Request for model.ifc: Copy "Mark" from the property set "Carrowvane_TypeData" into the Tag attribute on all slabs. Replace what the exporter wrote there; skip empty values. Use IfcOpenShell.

First a look at what the model holds.

```python
import ifcopenshell
import ifcopenshell.util.element

model = ifcopenshell.open("model.ifc")
print(model.schema)
slabs = model.by_type("IfcSlab")
print(len(slabs), "slabs")
for e in slabs[:8]:
    source = ifcopenshell.util.element.get_pset(e, "Carrowvane_TypeData", "Mark")
    target = e.Tag
    print(e.id(), repr(source), repr(target), sep=" | ")
```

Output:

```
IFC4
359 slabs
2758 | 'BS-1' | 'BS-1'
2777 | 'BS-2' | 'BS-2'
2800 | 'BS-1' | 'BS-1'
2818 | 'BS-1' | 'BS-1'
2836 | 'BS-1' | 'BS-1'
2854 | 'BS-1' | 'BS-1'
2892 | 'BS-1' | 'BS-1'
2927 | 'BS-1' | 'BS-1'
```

```python
import ifcopenshell
import ifcopenshell.util.element

model = ifcopenshell.open("model.ifc")

count = 0
for e in model.by_type("IfcSlab"):
    value = ifcopenshell.util.element.get_pset(e, "Carrowvane_TypeData", "Mark")
    current = e.Tag
    if not value or not value.strip() or current == value:
        continue
    e.Tag = value
    count += 1

print(count, "slabs updated")

model.write("model_rev.ifc")
```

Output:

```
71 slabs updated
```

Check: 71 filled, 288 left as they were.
